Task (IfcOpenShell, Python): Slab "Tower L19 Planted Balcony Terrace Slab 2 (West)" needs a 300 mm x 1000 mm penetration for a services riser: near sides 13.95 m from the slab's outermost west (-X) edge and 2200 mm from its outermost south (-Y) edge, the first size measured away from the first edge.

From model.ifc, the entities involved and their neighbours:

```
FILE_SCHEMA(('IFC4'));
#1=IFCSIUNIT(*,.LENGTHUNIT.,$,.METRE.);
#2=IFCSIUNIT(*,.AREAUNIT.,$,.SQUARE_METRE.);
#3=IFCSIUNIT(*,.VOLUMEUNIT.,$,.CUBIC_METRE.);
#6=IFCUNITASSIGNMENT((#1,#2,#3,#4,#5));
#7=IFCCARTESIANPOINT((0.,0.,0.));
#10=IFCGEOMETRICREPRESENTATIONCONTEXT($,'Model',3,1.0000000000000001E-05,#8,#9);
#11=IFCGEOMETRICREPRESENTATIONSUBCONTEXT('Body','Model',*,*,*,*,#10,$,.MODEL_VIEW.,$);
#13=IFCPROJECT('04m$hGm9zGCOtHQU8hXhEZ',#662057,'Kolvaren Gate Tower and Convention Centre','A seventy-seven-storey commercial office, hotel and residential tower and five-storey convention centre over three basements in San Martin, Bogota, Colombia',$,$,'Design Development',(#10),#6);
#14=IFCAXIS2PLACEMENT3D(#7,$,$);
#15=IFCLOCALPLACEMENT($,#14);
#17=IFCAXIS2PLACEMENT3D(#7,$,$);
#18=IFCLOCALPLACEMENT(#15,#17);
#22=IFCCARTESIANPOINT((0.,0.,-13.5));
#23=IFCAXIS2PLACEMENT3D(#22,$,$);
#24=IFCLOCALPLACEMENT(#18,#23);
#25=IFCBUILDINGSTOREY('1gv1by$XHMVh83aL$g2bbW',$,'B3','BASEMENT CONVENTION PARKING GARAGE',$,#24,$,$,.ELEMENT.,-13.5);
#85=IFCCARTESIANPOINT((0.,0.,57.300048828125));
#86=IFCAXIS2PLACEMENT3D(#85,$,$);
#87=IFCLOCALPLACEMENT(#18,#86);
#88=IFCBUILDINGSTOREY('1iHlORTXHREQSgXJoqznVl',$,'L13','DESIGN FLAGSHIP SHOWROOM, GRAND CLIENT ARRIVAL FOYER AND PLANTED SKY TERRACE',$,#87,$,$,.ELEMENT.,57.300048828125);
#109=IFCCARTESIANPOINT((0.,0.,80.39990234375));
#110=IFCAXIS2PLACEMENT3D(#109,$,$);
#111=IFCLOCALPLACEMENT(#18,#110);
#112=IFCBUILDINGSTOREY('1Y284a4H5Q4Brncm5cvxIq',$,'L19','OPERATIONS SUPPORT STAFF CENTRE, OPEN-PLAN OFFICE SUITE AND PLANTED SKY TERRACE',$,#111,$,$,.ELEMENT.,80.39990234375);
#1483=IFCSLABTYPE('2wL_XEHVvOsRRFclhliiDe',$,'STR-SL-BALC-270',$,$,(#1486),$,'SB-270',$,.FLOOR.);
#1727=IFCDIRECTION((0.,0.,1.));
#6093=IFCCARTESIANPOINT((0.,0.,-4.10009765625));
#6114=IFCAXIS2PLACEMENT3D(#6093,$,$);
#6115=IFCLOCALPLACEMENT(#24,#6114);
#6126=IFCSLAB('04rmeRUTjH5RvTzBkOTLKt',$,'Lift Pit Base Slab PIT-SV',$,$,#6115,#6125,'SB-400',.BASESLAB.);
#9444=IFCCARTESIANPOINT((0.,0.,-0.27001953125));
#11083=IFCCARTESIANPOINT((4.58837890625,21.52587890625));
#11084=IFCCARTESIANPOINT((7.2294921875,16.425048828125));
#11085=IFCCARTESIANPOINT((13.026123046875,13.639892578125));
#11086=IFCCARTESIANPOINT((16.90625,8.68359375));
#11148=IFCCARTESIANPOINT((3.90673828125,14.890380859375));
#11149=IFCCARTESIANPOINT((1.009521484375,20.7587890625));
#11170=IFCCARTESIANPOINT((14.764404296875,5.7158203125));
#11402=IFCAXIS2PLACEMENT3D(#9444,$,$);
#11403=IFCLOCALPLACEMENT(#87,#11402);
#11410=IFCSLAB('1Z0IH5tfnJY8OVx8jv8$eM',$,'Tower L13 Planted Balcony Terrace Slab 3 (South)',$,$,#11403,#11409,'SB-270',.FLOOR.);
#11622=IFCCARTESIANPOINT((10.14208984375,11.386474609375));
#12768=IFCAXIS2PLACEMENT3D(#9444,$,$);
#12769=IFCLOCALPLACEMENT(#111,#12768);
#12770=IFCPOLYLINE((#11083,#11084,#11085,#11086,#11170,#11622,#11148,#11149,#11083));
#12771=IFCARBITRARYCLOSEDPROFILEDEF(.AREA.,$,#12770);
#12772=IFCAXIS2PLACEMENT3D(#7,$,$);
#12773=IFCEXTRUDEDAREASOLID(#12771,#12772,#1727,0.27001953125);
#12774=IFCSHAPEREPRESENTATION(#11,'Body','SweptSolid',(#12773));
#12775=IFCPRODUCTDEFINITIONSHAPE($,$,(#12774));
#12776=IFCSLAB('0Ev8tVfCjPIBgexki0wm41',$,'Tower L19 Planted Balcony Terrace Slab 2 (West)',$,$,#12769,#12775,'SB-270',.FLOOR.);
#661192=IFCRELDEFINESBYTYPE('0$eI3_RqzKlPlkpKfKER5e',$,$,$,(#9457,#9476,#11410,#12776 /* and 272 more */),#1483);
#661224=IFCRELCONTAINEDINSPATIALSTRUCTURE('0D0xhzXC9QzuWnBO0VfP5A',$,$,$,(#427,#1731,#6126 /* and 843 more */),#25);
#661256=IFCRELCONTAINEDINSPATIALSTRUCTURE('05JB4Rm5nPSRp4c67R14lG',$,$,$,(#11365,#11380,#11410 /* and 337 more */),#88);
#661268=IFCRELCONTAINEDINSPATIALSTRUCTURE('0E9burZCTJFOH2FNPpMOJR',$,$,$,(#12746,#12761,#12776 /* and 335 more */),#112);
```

```python
import numpy as np
import ifcopenshell
import ifcopenshell.api.feature
import ifcopenshell.api.geometry
import ifcopenshell.api.root
import ifcopenshell.geom
import ifcopenshell.util.placement
import ifcopenshell.util.representation
import ifcopenshell.util.shape
import ifcopenshell.util.unit

model = ifcopenshell.open("model.ifc")
unit_scale = ifcopenshell.util.unit.calculate_unit_scale(model)
settings = ifcopenshell.geom.settings()


def volume(element):
    """Net volume in cubic metres, openings subtracted."""
    shape = ifcopenshell.geom.create_shape(settings, element)
    return ifcopenshell.util.shape.get_volume(shape.geometry)


slab = model.by_guid("0Ev8tVfCjPIBgexki0wm41")
before = volume(slab)

# Extent in the slab's own axes, in metres. The edges named are its -X and -Y sides.
slab_shape = ifcopenshell.geom.create_shape(settings, slab)
vertices = ifcopenshell.util.shape.get_vertices(slab_shape.geometry)
x_min, y_min, bottom = vertices.min(axis=0)
top = vertices[:, 2].max()

opening = ifcopenshell.api.root.create_entity(model, ifc_class="IfcOpeningElement", name="Services riser opening", predefined_type="OPENING")
context = ifcopenshell.util.representation.get_context(model, "Model", "Body", "MODEL_VIEW")
width, depth = 0.3, 1
outline = [(0.0, 0.0), (width, 0.0), (width, depth), (0.0, depth), (0.0, 0.0)]
# Overshoot both faces by 50 mm so the cut is clean.
shape = ifcopenshell.api.geometry.add_slab_representation(
    model, context=context, depth=top - bottom + 0.1, polyline=outline
)
ifcopenshell.api.geometry.assign_representation(model, product=opening, representation=shape)

matrix = ifcopenshell.util.placement.get_local_placement(slab.ObjectPlacement)
matrix[:, 3] = matrix @ np.append(np.array([x_min + 13.95, y_min + 2.2, bottom - 0.05]) / unit_scale, 1.0)
ifcopenshell.api.geometry.edit_object_placement(model, product=opening, matrix=matrix, is_si=False)
ifcopenshell.api.feature.add_feature(model, feature=opening, element=slab)

after = volume(slab)

print(f"slab volume {before:.3f} -> {after:.3f} m3")

model.write("model-out.ifc")
```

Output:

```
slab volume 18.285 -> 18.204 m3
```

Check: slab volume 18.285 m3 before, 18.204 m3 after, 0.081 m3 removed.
